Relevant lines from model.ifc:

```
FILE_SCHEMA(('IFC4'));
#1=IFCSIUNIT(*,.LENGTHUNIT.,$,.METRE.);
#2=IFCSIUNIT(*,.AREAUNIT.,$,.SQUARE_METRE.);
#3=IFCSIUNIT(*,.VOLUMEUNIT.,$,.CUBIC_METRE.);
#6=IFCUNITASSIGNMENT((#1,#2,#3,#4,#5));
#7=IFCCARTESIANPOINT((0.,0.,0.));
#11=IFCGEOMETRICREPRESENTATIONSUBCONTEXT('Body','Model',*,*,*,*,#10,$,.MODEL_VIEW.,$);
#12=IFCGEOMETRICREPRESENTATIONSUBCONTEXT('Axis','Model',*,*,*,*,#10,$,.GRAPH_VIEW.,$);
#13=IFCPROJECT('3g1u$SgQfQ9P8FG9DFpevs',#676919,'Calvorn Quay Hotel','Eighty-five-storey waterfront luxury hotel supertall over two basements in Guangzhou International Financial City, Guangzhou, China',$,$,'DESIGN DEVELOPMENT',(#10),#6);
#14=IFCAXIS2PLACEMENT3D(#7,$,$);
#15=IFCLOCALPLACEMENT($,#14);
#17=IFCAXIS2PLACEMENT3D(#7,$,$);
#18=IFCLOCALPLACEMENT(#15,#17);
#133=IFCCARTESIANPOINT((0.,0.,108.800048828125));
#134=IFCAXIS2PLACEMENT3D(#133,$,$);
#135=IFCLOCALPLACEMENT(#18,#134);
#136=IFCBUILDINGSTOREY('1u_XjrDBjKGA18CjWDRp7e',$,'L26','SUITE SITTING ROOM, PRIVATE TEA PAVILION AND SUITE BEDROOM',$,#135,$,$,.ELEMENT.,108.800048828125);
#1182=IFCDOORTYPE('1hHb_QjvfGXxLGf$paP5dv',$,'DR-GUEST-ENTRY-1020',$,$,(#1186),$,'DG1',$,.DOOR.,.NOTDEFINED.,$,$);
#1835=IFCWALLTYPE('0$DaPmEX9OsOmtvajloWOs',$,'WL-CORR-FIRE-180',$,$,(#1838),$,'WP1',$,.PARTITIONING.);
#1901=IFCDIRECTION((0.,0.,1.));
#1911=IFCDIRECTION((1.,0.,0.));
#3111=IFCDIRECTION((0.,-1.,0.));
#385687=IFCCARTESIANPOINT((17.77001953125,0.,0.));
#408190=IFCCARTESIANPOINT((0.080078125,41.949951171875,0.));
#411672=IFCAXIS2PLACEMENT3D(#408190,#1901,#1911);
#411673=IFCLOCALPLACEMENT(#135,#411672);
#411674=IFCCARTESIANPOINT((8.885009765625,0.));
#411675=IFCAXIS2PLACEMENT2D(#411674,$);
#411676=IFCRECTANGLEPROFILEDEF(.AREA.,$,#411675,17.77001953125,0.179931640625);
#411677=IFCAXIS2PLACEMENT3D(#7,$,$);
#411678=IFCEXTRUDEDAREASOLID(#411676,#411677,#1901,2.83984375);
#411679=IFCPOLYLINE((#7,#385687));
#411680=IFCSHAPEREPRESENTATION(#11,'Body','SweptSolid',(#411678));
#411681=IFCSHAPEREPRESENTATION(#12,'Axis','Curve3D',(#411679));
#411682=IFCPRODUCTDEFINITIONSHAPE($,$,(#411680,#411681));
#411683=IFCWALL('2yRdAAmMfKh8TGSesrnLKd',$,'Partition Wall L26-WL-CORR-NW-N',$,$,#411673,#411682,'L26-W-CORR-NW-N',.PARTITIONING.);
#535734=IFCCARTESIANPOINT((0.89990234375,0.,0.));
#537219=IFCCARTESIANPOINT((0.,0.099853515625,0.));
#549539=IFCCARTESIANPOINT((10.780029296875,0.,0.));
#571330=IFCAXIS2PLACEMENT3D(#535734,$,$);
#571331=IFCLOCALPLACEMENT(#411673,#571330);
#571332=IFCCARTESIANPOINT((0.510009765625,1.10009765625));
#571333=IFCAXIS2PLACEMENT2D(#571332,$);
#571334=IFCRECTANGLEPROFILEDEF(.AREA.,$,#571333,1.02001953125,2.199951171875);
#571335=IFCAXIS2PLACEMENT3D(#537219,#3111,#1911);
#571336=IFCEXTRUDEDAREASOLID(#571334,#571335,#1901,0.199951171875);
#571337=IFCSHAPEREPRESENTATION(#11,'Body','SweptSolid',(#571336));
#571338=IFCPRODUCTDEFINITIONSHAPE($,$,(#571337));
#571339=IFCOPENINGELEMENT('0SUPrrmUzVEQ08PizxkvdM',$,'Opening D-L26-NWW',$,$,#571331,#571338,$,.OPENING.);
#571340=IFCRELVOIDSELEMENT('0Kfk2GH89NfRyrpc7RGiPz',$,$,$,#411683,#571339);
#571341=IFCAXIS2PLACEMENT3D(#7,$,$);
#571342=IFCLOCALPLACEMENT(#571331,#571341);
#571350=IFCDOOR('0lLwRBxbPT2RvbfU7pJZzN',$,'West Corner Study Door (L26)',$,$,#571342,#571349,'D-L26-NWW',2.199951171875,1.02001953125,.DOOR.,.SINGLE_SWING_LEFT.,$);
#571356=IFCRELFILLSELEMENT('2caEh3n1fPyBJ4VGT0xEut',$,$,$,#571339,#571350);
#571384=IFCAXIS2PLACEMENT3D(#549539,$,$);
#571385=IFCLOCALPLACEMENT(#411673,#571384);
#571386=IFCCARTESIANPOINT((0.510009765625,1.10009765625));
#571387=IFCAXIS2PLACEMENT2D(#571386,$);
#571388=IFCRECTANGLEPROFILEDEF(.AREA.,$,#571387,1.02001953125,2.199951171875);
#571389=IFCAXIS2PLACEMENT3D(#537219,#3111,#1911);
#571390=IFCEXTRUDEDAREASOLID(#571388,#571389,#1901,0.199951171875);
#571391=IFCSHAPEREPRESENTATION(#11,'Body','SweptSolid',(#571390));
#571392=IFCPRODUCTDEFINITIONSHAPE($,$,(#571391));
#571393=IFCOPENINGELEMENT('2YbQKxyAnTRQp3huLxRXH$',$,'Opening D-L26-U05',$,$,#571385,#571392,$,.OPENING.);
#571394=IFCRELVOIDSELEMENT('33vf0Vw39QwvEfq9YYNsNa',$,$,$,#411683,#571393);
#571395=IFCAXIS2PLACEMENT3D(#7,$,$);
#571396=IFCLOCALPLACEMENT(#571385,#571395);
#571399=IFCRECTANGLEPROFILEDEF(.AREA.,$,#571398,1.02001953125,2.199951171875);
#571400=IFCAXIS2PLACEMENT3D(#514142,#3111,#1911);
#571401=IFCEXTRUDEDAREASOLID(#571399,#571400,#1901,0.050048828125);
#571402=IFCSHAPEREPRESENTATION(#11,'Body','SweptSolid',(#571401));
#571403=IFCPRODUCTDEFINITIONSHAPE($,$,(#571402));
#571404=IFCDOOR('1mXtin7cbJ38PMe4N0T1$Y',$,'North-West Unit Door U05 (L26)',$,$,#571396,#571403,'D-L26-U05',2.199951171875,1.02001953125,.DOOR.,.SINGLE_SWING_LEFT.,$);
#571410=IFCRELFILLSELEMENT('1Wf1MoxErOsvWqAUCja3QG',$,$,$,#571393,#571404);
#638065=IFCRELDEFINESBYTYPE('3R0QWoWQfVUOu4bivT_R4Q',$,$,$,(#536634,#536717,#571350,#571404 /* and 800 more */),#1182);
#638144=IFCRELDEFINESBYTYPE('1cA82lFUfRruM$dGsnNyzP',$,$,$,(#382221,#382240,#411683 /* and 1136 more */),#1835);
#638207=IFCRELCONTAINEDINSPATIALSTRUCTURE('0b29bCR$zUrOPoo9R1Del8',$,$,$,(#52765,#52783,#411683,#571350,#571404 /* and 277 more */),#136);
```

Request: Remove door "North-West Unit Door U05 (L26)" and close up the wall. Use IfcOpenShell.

```python
import ifcopenshell
import ifcopenshell.api.feature
import ifcopenshell.api.root
import ifcopenshell.geom
import ifcopenshell.util.shape

model = ifcopenshell.open("model.ifc")
settings = ifcopenshell.geom.settings()


def volume(element):
    """Net volume in cubic metres, openings subtracted."""
    shape = ifcopenshell.geom.create_shape(settings, element)
    return ifcopenshell.util.shape.get_volume(shape.geometry)


door = model.by_id(571404)
opening = door.FillsVoids[0].RelatingOpeningElement
wall = opening.VoidsElements[0].RelatingBuildingElement
before = volume(wall)

ifcopenshell.api.root.remove_product(model, product=door)
ifcopenshell.api.feature.remove_feature(model, feature=opening)

after = volume(wall)

print(f"wall volume {before:.3f} -> {after:.3f} m3")

model.write("model_edited.ifc")
```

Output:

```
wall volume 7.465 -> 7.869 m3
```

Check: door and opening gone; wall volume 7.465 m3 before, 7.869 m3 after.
